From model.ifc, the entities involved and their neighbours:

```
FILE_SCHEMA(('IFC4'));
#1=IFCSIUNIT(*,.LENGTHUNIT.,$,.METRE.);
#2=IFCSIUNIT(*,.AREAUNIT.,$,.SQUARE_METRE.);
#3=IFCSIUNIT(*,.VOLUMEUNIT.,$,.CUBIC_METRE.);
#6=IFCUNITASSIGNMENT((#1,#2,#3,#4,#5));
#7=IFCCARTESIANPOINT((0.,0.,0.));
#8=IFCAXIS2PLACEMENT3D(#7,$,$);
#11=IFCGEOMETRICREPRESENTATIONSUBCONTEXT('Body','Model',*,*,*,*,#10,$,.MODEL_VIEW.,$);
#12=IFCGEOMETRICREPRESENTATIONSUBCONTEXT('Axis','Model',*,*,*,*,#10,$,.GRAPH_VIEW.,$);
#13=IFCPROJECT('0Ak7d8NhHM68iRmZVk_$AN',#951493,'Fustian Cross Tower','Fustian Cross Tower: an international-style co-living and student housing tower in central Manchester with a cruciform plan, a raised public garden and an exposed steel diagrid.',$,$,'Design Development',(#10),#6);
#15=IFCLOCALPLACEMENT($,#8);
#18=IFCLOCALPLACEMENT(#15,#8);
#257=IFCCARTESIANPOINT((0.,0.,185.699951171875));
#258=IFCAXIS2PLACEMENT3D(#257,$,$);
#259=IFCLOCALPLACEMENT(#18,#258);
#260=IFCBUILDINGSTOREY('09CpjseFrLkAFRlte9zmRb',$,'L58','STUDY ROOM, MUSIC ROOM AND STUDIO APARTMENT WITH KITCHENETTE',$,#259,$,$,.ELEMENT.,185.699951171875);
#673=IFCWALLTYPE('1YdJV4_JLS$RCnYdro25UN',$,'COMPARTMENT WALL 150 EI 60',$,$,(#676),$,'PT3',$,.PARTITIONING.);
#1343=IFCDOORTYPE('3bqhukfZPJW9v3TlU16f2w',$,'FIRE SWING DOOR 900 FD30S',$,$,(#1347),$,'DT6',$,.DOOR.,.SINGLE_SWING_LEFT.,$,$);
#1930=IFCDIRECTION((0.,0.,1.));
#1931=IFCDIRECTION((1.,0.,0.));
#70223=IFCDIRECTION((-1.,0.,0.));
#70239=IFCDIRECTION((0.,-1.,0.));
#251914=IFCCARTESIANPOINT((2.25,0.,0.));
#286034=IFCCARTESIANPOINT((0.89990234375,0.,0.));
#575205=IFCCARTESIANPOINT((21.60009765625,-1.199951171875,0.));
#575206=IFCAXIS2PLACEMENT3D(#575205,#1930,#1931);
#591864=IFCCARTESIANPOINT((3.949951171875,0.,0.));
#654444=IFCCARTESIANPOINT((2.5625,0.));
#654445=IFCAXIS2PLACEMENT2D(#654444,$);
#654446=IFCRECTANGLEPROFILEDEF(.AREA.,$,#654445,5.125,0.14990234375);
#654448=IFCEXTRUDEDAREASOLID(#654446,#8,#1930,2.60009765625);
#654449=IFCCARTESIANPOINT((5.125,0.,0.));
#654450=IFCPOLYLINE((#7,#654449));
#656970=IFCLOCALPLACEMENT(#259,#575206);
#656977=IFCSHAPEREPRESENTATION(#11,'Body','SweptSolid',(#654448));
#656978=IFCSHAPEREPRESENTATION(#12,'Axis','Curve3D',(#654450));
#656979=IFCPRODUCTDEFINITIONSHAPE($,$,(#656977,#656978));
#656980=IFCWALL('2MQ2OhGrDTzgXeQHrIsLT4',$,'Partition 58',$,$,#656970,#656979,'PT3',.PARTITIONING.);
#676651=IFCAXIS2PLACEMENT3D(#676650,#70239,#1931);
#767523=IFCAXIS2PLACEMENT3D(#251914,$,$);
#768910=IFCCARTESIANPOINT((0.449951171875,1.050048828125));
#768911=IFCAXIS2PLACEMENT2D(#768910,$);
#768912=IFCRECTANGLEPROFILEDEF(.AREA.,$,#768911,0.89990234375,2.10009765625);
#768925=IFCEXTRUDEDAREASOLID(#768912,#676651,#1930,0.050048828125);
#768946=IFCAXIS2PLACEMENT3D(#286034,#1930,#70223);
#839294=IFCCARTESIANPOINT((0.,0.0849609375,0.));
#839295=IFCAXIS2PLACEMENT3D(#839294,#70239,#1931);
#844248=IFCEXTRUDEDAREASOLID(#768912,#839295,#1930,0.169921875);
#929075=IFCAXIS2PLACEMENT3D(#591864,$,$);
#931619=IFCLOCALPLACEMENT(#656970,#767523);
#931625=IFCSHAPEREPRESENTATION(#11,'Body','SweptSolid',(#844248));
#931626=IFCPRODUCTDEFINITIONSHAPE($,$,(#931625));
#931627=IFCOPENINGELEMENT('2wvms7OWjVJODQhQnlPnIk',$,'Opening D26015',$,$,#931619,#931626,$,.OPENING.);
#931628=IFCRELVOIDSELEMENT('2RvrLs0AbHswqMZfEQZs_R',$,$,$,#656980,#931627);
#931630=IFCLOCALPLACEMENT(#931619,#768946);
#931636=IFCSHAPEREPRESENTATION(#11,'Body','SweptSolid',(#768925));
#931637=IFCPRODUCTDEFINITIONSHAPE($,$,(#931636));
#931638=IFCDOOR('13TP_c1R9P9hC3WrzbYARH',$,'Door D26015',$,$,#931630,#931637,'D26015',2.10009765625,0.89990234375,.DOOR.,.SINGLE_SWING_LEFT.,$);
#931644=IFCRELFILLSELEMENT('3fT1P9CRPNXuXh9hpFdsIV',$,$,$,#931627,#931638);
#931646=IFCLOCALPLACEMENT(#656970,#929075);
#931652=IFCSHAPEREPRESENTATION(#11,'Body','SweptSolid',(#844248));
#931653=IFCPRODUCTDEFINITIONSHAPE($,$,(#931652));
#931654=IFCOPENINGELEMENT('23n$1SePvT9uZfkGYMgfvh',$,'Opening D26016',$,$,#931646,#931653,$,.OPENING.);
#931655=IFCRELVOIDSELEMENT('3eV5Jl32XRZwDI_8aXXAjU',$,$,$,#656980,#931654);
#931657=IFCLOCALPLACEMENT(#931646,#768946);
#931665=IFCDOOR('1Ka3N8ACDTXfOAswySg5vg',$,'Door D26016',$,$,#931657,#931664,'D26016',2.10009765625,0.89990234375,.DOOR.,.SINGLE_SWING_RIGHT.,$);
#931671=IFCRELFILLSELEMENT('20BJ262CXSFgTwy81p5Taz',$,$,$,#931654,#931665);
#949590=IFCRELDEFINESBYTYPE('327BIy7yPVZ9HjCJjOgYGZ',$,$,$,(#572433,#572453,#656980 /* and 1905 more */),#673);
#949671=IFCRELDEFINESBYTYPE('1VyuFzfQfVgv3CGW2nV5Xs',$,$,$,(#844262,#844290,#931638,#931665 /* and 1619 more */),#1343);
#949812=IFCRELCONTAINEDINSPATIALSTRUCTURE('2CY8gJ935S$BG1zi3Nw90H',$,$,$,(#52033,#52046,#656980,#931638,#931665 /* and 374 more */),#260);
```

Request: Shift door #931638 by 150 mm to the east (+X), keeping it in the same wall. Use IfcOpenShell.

```python
import ifcopenshell
import ifcopenshell.api.geometry
import ifcopenshell.util.placement

model = ifcopenshell.open("model.ifc")

door = model.by_guid("13TP_c1R9P9hC3WrzbYARH")
opening = door.FillsVoids[0].RelatingOpeningElement
wall = opening.VoidsElements[0].RelatingBuildingElement

wall_matrix = ifcopenshell.util.placement.get_local_placement(wall.ObjectPlacement)
shift = wall_matrix[:3, 0] * 0.15
before = ifcopenshell.util.placement.get_local_placement(door.ObjectPlacement)[:3, 3].copy()

# The door is placed relative to its opening, so it follows when the opening moves.
matrix = ifcopenshell.util.placement.get_local_placement(opening.ObjectPlacement)
matrix[:3, 3] += shift
ifcopenshell.api.geometry.edit_object_placement(
    model, product=opening, matrix=matrix, is_si=False, should_transform_children=True
)

after = ifcopenshell.util.placement.get_local_placement(door.ObjectPlacement)[:3, 3]
print("door moved by", (after - before).round(3) + 0.0)

model.write("model-out.ifc")
```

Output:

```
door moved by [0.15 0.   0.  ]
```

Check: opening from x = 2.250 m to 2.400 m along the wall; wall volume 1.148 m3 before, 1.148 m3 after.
